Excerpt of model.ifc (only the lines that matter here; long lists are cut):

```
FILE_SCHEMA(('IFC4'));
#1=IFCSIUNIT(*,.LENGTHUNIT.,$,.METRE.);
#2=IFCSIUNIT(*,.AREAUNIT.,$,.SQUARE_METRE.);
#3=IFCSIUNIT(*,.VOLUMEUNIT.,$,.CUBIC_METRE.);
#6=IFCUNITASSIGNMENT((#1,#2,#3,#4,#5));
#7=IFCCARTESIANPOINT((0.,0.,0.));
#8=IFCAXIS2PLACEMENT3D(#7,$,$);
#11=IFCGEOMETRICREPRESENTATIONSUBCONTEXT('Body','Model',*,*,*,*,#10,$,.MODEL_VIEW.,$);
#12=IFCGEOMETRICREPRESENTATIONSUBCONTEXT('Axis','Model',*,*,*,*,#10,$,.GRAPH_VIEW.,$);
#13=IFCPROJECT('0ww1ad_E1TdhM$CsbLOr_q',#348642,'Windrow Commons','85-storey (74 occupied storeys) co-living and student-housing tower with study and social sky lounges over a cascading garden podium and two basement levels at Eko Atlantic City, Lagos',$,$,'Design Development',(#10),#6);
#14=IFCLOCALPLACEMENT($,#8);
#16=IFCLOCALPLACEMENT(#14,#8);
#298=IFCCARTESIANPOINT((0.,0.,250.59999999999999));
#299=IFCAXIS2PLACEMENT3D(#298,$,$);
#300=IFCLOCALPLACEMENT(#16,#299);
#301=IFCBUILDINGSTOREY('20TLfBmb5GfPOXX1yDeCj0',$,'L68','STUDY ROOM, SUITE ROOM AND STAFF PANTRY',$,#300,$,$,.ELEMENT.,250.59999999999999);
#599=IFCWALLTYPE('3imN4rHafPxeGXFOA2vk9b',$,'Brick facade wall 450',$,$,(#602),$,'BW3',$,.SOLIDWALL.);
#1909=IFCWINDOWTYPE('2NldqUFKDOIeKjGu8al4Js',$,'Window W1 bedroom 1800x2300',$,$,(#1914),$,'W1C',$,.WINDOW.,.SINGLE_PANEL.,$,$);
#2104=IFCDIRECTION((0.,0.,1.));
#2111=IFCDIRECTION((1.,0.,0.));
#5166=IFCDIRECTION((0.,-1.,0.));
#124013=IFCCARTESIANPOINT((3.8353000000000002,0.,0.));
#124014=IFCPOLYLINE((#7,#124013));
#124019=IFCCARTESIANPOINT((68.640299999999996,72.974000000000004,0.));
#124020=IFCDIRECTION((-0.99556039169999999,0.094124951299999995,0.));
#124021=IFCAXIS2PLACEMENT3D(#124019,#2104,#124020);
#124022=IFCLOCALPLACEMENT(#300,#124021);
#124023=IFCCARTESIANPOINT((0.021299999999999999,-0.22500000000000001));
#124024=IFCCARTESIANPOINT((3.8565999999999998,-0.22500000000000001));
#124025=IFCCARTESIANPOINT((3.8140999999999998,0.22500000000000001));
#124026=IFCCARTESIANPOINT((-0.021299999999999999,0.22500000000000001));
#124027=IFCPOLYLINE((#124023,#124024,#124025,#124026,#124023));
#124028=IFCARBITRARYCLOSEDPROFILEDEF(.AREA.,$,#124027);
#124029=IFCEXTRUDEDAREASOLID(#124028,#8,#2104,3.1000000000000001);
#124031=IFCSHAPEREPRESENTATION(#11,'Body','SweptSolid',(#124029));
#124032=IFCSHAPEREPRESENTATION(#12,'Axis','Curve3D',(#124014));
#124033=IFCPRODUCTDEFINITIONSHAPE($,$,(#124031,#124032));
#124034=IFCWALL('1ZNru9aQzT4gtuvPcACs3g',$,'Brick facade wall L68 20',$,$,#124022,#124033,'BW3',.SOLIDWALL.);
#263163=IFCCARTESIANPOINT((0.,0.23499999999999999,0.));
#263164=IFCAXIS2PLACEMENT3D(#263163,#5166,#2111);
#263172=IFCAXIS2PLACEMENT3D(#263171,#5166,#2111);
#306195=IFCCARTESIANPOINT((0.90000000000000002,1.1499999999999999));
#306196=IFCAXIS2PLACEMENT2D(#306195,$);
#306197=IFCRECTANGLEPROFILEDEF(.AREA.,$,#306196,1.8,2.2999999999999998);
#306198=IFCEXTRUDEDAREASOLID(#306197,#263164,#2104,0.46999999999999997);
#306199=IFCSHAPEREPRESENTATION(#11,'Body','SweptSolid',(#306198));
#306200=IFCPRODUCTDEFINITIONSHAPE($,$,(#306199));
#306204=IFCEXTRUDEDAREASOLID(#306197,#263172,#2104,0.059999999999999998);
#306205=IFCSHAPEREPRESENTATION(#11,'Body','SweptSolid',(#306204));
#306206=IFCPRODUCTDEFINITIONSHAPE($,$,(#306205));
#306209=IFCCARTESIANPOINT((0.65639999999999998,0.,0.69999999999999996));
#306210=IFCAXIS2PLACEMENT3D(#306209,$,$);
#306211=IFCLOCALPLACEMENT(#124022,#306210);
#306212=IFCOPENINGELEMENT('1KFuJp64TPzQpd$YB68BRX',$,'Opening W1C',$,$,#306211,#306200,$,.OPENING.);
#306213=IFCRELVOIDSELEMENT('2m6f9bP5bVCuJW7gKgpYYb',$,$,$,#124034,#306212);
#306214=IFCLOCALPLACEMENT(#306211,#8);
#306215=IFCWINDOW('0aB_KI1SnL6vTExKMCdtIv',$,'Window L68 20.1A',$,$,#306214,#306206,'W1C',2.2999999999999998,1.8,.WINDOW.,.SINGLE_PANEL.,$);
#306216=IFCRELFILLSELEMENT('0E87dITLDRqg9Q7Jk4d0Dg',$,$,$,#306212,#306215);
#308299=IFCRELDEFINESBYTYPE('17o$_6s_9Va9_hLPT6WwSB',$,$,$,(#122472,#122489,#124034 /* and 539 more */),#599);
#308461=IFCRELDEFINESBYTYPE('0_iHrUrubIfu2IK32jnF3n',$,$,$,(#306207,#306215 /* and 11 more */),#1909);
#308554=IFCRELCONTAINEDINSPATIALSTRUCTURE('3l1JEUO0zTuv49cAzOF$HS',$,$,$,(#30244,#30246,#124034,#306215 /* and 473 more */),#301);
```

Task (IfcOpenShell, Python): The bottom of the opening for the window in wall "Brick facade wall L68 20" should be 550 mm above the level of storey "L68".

```python
import numpy as np
import ifcopenshell
import ifcopenshell.api.geometry
import ifcopenshell.geom
import ifcopenshell.util.element
import ifcopenshell.util.placement
import ifcopenshell.util.shape
import ifcopenshell.util.unit

model = ifcopenshell.open("model.ifc")
unit_scale = ifcopenshell.util.unit.calculate_unit_scale(model)

window = model.by_guid("0aB_KI1SnL6vTExKMCdtIv")
opening = window.FillsVoids[0].RelatingOpeningElement
storey = ifcopenshell.util.element.get_container(window, ifc_class="IfcBuildingStorey")
level = ifcopenshell.util.placement.get_local_placement(storey.ObjectPlacement)[2, 3]

# The opening's origin need not be at the sill, so measure its lowest point.
shape = ifcopenshell.geom.create_shape(ifcopenshell.geom.settings(), opening)
bottom = ifcopenshell.util.shape.get_shape_bottom_elevation(shape, shape.geometry) / unit_scale
dz = level + 0.55 / unit_scale - bottom

shift = np.array([0.0, 0.0, dz])
# The window is placed relative to its opening, so it follows when the opening moves.
matrix = ifcopenshell.util.placement.get_local_placement(opening.ObjectPlacement)
matrix[:3, 3] += shift
ifcopenshell.api.geometry.edit_object_placement(
    model, product=opening, matrix=matrix, is_si=False, should_transform_children=True
)

print(f"moved by {dz * unit_scale:+.3f} m")

model.write("model_rev.ifc")
```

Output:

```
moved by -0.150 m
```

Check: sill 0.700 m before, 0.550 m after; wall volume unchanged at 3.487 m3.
